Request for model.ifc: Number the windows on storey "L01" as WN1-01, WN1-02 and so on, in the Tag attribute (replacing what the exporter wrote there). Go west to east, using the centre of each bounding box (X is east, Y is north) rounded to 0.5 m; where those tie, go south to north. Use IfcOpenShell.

First a look at what the model holds.

```python
import ifcopenshell
import ifcopenshell.util.element
import ifcopenshell.util.placement

model = ifcopenshell.open("model.ifc")
print(model.schema)
storey = next(s for s in model.by_type("IfcBuildingStorey") if s.Name == "L01")
windows = [e for e in ifcopenshell.util.element.get_decomposition(storey) if e.is_a("IfcWindow")]
for e in sorted(windows, key=lambda e: e.id()):
    origin = ifcopenshell.util.placement.get_local_placement(e.ObjectPlacement)[:3, 3]
    print(e.id(), e.Tag, e.Name, origin.round(2) + 0.0, sep=" | ")
```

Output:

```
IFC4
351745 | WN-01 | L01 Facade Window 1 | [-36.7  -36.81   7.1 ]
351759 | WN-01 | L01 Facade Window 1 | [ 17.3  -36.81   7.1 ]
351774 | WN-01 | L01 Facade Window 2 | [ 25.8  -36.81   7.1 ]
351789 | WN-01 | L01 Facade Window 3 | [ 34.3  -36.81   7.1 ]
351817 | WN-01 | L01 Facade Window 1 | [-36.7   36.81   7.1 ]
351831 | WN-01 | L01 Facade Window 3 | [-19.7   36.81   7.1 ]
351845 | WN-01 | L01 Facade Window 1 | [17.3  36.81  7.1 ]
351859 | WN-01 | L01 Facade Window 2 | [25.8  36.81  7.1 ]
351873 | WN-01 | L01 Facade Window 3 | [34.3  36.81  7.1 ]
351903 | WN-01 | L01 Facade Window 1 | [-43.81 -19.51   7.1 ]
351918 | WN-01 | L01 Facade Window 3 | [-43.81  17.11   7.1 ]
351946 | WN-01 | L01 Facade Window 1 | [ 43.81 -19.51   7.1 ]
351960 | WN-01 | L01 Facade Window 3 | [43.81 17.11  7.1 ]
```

```python
import ifcopenshell
import ifcopenshell.geom
import ifcopenshell.util.element
import ifcopenshell.util.shape

model = ifcopenshell.open("model.ifc")
settings = ifcopenshell.geom.settings()
settings.set("use-world-coords", True)


def centre(element):
    shape = ifcopenshell.geom.create_shape(settings, element)
    return ifcopenshell.util.shape.get_bbox_centroid(shape.geometry)


storey = next(s for s in model.by_type("IfcBuildingStorey") if s.Name == "L01")
windows = [e for e in ifcopenshell.util.element.get_decomposition(storey) if e.is_a("IfcWindow")]

# Insertion points can sit at a corner or the storey origin, so sort by the geometry (in metres).
centres = {e: centre(e) for e in windows}
windows.sort(key=lambda e: (round(centres[e][0] / 0.5), centres[e][1]))

for i, e in enumerate(windows, start=1):
    number = f"WN1-{i:02d}"
    e.Tag = number
    print(e.id(), number)

model.write("model_edited.ifc")
```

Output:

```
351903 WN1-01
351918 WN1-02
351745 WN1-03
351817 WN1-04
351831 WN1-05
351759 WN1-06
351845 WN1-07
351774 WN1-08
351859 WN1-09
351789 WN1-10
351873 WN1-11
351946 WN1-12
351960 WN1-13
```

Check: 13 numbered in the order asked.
